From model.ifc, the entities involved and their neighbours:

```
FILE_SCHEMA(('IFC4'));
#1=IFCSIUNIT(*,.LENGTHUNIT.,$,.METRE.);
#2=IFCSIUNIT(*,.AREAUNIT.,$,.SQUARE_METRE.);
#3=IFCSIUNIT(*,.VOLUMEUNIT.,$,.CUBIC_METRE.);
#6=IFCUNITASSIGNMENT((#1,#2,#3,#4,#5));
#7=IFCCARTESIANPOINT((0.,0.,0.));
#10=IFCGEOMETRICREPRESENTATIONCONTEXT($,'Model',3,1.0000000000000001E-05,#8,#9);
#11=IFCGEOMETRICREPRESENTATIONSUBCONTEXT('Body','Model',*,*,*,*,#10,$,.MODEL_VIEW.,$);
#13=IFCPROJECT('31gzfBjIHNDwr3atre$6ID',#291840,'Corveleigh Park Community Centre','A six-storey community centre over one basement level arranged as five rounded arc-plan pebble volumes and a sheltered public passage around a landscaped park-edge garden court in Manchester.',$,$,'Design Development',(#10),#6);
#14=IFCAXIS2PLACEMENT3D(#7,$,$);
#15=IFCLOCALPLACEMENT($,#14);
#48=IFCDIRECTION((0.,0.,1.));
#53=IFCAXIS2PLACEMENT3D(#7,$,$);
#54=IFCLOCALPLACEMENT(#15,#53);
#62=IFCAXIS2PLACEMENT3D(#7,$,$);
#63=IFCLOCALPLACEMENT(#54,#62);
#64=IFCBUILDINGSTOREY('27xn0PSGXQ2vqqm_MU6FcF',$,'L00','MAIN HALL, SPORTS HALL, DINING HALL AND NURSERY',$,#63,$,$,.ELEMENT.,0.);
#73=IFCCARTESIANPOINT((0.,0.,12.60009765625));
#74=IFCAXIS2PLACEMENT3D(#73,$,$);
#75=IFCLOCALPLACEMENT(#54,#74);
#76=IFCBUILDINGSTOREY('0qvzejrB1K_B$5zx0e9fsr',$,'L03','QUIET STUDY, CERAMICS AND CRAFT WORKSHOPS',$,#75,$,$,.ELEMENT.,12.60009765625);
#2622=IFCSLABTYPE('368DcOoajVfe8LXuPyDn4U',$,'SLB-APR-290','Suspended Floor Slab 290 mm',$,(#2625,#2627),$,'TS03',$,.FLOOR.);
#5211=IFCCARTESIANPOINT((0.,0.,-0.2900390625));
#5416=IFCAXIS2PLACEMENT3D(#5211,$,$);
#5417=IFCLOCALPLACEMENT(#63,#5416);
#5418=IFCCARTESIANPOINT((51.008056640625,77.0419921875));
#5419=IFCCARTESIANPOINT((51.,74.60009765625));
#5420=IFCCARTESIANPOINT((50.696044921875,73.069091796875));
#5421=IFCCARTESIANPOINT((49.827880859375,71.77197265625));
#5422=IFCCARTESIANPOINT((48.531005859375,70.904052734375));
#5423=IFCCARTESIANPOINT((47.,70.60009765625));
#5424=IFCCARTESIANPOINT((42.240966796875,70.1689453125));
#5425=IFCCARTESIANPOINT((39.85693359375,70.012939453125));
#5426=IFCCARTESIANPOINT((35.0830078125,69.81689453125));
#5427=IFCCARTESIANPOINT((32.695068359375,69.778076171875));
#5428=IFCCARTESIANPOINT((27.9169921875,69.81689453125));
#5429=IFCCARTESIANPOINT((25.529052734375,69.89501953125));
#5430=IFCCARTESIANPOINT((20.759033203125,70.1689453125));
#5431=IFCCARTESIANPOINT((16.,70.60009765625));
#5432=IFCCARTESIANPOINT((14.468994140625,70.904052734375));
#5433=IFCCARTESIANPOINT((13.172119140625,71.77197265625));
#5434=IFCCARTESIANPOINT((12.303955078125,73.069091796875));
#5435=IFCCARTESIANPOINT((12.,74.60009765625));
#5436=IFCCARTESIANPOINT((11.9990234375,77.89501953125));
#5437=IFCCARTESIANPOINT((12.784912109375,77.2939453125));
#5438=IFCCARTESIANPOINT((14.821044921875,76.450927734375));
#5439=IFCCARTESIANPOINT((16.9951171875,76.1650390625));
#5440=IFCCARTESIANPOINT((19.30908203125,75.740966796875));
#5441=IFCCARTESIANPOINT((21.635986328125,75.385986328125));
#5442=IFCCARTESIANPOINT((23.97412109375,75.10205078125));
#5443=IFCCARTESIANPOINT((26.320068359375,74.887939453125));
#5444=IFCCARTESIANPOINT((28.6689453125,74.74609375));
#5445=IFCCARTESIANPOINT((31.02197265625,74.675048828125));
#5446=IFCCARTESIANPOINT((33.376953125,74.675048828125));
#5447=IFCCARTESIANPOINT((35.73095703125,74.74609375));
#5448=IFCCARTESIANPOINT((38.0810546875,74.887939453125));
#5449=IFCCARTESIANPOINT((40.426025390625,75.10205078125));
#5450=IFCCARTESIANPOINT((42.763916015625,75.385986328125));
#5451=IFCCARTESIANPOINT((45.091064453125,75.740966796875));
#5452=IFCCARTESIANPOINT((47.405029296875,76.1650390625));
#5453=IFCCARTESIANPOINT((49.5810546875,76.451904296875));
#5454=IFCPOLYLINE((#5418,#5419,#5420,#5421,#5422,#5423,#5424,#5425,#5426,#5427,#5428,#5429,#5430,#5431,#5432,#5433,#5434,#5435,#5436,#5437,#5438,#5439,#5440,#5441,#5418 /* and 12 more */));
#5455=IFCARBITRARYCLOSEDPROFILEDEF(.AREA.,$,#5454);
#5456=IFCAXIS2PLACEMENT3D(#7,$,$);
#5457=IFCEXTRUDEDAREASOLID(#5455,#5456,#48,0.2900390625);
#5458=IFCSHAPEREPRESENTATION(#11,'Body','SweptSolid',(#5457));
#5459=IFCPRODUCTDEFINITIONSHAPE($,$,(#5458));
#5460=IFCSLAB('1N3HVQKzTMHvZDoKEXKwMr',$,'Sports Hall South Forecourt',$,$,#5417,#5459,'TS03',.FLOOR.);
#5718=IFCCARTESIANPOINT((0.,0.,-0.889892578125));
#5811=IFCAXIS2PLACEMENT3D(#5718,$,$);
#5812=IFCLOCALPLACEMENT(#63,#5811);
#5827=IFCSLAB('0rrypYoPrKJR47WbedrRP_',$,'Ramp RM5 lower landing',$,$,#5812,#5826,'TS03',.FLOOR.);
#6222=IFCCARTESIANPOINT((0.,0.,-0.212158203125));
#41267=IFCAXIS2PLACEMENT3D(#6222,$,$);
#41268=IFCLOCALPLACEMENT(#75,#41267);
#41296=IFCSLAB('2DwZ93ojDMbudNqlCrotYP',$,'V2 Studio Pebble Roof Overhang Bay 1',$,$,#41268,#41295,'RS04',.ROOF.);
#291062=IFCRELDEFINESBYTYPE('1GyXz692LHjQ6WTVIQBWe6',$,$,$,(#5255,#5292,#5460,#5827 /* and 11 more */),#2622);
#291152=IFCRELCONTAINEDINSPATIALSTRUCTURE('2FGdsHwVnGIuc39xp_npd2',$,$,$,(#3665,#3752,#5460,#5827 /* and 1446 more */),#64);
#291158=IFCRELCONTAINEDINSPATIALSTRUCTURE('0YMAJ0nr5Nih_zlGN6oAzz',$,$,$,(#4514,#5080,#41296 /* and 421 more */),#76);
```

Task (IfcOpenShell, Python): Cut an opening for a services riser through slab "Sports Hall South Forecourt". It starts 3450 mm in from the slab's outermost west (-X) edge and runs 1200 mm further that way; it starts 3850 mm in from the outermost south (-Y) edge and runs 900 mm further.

```python
import numpy as np
import ifcopenshell
import ifcopenshell.api.feature
import ifcopenshell.api.geometry
import ifcopenshell.api.root
import ifcopenshell.geom
import ifcopenshell.util.placement
import ifcopenshell.util.representation
import ifcopenshell.util.shape
import ifcopenshell.util.unit

model = ifcopenshell.open("model.ifc")
unit_scale = ifcopenshell.util.unit.calculate_unit_scale(model)
settings = ifcopenshell.geom.settings()


def volume(element):
    """Net volume in cubic metres, openings subtracted."""
    shape = ifcopenshell.geom.create_shape(settings, element)
    return ifcopenshell.util.shape.get_volume(shape.geometry)


slab = model.by_guid("1N3HVQKzTMHvZDoKEXKwMr")
before = volume(slab)

# Extent in the slab's own axes, in metres. The edges named are its -X and -Y sides.
slab_shape = ifcopenshell.geom.create_shape(settings, slab)
vertices = ifcopenshell.util.shape.get_vertices(slab_shape.geometry)
x_min, y_min, bottom = vertices.min(axis=0)
top = vertices[:, 2].max()

opening = ifcopenshell.api.root.create_entity(model, ifc_class="IfcOpeningElement", name="Services riser opening", predefined_type="OPENING")
context = ifcopenshell.util.representation.get_context(model, "Model", "Body", "MODEL_VIEW")
width, depth = 1.2, 0.9
outline = [(0.0, 0.0), (width, 0.0), (width, depth), (0.0, depth), (0.0, 0.0)]
# Overshoot both faces by 50 mm so the cut is clean.
shape = ifcopenshell.api.geometry.add_slab_representation(
    model, context=context, depth=top - bottom + 0.1, polyline=outline
)
ifcopenshell.api.geometry.assign_representation(model, product=opening, representation=shape)

matrix = ifcopenshell.util.placement.get_local_placement(slab.ObjectPlacement)
matrix[:, 3] = matrix @ np.append(np.array([x_min + 3.45, y_min + 3.85, bottom - 0.05]) / unit_scale, 1.0)
ifcopenshell.api.geometry.edit_object_placement(model, product=opening, matrix=matrix, is_si=False)
ifcopenshell.api.feature.add_feature(model, feature=opening, element=slab)

after = volume(slab)

print(f"slab volume {before:.3f} -> {after:.3f} m3")

model.write("model_edited.ifc")
```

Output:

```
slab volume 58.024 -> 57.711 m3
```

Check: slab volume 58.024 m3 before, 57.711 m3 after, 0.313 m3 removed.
